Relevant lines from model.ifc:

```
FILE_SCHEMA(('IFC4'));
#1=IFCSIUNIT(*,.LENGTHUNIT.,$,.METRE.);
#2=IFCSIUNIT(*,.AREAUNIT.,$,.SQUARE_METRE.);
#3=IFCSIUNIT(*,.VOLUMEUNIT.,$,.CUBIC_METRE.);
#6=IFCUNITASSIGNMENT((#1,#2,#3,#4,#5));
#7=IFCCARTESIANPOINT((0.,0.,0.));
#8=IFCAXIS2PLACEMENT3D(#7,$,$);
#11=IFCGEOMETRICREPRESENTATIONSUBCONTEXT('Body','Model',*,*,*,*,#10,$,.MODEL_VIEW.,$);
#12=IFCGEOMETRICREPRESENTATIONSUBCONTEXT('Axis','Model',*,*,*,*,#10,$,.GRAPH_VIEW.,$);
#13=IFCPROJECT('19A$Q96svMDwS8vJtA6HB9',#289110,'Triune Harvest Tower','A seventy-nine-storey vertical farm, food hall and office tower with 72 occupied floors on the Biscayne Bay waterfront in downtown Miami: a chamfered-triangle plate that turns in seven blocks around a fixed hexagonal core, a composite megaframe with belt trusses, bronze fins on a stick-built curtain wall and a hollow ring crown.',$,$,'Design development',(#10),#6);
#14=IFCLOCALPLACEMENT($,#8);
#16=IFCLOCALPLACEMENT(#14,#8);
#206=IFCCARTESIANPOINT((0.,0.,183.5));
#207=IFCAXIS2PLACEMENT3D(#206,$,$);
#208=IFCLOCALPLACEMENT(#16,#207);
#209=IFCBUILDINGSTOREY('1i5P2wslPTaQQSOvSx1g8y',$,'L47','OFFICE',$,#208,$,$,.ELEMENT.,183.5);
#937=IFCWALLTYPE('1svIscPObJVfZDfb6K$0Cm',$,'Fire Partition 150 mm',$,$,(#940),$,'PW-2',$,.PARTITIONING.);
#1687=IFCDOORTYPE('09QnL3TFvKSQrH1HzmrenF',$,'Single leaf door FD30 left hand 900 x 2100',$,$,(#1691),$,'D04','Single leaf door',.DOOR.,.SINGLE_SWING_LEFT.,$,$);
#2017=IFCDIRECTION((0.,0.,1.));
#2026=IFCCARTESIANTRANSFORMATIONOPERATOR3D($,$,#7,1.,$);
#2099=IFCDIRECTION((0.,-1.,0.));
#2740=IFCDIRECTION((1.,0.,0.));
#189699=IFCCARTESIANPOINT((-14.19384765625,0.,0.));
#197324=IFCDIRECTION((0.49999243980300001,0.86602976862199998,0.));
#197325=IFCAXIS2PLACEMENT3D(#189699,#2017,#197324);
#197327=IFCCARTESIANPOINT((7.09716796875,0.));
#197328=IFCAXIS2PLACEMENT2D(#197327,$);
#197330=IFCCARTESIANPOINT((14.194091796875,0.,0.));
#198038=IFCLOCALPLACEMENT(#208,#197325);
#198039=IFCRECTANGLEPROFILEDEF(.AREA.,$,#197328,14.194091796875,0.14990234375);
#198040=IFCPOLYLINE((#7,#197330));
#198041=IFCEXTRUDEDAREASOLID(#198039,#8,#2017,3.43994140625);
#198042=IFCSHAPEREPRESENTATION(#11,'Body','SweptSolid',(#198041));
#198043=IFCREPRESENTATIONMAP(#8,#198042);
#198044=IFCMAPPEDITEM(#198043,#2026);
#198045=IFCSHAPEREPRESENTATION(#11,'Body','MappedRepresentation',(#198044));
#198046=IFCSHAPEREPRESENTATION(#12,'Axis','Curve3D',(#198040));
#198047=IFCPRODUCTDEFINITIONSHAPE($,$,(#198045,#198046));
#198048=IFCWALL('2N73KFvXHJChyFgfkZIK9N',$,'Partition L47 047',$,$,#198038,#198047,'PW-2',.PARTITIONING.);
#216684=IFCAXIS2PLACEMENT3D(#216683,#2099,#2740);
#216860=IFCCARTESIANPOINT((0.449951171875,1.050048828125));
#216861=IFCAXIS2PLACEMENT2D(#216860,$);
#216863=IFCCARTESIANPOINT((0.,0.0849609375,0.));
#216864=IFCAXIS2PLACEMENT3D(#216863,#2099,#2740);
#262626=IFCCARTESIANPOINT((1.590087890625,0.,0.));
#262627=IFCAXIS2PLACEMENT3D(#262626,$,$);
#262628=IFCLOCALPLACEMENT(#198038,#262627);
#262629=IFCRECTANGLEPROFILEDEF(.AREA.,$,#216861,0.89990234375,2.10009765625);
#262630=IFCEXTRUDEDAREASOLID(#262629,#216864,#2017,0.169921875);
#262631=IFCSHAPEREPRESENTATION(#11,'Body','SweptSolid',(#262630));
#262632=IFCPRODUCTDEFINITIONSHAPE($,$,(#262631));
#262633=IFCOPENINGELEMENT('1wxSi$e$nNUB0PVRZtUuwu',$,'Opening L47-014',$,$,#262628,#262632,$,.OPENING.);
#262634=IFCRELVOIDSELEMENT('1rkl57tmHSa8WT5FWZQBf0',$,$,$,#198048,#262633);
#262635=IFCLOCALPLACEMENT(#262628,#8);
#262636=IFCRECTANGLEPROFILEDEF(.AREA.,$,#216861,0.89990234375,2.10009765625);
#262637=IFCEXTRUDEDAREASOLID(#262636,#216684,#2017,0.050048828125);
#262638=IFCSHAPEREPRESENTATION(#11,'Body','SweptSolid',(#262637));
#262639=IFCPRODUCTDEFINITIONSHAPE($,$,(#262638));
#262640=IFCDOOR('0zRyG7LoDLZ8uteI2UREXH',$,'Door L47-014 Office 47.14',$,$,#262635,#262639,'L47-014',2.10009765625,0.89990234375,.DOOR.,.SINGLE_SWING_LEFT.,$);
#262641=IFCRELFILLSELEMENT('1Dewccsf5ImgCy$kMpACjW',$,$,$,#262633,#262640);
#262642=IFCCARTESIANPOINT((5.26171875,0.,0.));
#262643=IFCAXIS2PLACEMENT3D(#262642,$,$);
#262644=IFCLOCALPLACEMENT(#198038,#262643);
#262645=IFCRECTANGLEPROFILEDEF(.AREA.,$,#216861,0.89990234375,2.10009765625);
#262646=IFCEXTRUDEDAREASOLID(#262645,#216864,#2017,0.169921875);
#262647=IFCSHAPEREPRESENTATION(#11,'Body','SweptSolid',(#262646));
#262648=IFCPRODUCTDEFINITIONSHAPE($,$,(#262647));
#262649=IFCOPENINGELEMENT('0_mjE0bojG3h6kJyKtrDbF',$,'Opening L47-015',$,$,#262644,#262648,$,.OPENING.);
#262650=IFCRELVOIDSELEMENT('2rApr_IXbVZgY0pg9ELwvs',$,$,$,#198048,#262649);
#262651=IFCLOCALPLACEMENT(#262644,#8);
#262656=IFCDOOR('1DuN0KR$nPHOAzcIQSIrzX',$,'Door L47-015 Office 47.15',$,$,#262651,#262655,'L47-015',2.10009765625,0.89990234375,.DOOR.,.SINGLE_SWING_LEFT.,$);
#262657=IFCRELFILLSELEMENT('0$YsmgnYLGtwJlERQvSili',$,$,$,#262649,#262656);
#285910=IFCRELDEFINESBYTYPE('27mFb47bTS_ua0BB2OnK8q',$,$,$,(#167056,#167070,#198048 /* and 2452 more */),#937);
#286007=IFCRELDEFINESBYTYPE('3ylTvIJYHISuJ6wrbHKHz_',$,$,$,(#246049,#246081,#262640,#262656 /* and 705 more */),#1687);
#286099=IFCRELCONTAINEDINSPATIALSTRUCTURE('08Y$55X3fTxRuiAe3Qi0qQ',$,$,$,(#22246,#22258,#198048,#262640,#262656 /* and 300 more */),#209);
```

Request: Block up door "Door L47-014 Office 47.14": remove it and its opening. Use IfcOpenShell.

```python
import ifcopenshell
import ifcopenshell.api.feature
import ifcopenshell.api.root
import ifcopenshell.geom
import ifcopenshell.util.shape

model = ifcopenshell.open("model.ifc")
settings = ifcopenshell.geom.settings()


def volume(element):
    """Net volume in cubic metres, openings subtracted."""
    shape = ifcopenshell.geom.create_shape(settings, element)
    return ifcopenshell.util.shape.get_volume(shape.geometry)


door = model.by_id(262640)
opening = door.FillsVoids[0].RelatingOpeningElement
wall = opening.VoidsElements[0].RelatingBuildingElement
before = volume(wall)

ifcopenshell.api.root.remove_product(model, product=door)
ifcopenshell.api.feature.remove_feature(model, feature=opening)

after = volume(wall)

print(f"wall volume {before:.3f} -> {after:.3f} m3")

model.write("model_edited.ifc")
```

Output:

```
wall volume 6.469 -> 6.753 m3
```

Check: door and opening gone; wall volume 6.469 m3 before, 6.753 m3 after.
